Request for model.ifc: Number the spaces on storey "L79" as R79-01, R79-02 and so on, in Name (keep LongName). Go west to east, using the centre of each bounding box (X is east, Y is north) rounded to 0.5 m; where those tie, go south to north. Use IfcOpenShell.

First a look at what the model holds.

```python
import ifcopenshell
import ifcopenshell.util.element
import ifcopenshell.util.placement

model = ifcopenshell.open("model.ifc")
print(model.schema)
storey = next(s for s in model.by_type("IfcBuildingStorey") if s.Name == "L79")
spaces = [e for e in ifcopenshell.util.element.get_decomposition(storey) if e.is_a("IfcSpace")]
for e in sorted(spaces, key=lambda e: e.id()):
    origin = ifcopenshell.util.placement.get_local_placement(e.ObjectPlacement)[:3, 3]
    print(e.id(), e.Name, e.LongName, origin.round(2) + 0.0, sep=" | ")
```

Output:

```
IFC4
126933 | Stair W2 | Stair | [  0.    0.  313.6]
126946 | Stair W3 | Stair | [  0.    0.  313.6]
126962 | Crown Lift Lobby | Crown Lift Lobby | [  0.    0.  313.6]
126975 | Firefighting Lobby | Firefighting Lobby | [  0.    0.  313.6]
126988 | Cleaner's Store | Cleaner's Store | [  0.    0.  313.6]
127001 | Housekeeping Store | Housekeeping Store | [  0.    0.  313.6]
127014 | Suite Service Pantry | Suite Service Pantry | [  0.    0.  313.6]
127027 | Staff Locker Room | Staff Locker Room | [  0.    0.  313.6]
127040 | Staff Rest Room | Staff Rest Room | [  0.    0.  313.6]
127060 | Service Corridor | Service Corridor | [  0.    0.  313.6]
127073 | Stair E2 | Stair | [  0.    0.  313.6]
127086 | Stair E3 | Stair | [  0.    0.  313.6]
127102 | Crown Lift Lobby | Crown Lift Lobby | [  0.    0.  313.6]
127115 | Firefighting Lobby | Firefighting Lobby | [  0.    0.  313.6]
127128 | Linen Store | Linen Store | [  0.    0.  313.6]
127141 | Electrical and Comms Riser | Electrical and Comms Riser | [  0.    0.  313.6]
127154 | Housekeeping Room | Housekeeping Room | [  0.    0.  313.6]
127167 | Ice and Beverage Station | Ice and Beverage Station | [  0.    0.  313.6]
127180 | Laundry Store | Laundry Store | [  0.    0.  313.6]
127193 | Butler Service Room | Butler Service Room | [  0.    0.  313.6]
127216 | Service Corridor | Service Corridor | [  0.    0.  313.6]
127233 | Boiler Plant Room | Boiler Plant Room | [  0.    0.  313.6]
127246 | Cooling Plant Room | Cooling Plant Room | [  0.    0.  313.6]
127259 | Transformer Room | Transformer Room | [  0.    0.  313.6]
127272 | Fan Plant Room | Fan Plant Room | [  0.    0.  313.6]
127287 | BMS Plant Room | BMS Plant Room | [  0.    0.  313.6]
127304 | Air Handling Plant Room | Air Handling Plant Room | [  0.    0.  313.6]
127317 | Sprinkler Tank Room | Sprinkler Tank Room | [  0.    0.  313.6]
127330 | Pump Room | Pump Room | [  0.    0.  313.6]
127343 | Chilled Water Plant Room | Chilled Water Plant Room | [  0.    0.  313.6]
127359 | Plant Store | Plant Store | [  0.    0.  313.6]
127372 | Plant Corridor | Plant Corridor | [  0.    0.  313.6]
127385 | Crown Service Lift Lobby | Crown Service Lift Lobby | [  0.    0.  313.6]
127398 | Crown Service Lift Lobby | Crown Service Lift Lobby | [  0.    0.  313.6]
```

```python
import ifcopenshell
import ifcopenshell.geom
import ifcopenshell.util.element
import ifcopenshell.util.shape

model = ifcopenshell.open("model.ifc")
settings = ifcopenshell.geom.settings()
settings.set("use-world-coords", True)


def centre(element):
    shape = ifcopenshell.geom.create_shape(settings, element)
    return ifcopenshell.util.shape.get_bbox_centroid(shape.geometry)


storey = next(s for s in model.by_type("IfcBuildingStorey") if s.Name == "L79")
spaces = [e for e in ifcopenshell.util.element.get_decomposition(storey) if e.is_a("IfcSpace")]

# Insertion points can sit at a corner or the storey origin, so sort by the geometry (in metres).
centres = {e: centre(e) for e in spaces}
spaces.sort(key=lambda e: (round(centres[e][0] / 0.5), centres[e][1]))

for i, e in enumerate(spaces, start=1):
    number = f"R79-{i:02d}"
    e.Name = number
    print(e.id(), number)

model.write("model_rev.ifc")
```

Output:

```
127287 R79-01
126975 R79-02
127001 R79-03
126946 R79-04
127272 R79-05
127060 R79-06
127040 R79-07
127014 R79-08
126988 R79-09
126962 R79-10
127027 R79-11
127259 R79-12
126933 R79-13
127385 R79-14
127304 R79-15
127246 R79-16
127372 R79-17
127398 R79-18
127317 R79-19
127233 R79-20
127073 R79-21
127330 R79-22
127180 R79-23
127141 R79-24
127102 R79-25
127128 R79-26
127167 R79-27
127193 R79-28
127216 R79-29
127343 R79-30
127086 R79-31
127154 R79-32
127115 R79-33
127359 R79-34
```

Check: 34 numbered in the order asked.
